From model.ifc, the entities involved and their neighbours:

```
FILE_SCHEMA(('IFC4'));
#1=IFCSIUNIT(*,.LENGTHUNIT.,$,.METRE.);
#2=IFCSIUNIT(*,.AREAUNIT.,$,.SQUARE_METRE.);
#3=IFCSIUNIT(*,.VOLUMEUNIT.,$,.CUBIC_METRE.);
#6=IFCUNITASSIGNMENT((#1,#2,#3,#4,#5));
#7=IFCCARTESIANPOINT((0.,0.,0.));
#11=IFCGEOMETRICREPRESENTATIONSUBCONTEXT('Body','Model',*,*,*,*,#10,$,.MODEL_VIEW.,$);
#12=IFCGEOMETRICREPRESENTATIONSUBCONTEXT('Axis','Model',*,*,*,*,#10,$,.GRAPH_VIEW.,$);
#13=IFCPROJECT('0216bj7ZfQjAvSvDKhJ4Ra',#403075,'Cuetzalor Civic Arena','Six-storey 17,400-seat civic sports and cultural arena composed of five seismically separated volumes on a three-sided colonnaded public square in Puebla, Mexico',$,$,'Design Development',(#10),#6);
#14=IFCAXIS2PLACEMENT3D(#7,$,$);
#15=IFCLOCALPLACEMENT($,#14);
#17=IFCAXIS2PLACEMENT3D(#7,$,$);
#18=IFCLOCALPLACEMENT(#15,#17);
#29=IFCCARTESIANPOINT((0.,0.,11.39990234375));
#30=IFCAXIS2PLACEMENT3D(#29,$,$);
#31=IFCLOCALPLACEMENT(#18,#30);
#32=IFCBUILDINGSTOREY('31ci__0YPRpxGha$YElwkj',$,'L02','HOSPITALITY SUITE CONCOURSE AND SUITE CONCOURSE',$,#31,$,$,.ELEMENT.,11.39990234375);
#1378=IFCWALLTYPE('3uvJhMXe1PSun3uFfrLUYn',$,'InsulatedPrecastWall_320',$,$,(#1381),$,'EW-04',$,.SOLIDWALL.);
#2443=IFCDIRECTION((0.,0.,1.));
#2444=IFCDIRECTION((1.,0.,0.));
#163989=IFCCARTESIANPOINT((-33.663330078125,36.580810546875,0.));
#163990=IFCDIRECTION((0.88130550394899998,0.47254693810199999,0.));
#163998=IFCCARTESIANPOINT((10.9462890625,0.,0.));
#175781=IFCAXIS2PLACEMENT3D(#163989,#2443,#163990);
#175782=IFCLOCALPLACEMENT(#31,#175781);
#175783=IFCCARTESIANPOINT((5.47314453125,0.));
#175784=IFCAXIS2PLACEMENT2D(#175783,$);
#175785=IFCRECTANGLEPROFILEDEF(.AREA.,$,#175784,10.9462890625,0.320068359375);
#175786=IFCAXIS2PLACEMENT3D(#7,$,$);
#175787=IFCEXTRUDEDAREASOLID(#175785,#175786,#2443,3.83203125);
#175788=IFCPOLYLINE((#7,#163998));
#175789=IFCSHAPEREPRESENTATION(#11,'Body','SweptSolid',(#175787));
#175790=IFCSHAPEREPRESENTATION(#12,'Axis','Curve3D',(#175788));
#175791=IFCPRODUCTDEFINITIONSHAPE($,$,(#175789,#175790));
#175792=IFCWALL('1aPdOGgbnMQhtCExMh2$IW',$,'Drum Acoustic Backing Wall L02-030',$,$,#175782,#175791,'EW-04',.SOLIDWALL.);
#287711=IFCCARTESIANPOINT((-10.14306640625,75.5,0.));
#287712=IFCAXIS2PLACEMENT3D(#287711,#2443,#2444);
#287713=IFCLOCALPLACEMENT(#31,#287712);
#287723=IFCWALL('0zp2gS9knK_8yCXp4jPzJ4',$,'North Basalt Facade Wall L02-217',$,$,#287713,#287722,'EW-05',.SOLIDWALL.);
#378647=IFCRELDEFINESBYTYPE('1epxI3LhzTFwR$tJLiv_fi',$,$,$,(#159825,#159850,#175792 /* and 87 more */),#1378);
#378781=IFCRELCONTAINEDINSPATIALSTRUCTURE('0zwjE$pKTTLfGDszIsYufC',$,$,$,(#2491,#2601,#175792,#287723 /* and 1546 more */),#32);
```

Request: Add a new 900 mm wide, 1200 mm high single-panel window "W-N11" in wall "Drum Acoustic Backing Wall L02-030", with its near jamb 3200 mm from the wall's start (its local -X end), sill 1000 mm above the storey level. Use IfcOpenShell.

```python
import numpy as np
import ifcopenshell
import ifcopenshell.api.feature
import ifcopenshell.api.geometry
import ifcopenshell.api.root
import ifcopenshell.api.spatial
import ifcopenshell.geom
import ifcopenshell.util.element
import ifcopenshell.util.placement
import ifcopenshell.util.representation
import ifcopenshell.util.shape
import ifcopenshell.util.unit

model = ifcopenshell.open("model.ifc")
unit_scale = ifcopenshell.util.unit.calculate_unit_scale(model)
settings = ifcopenshell.geom.settings()


def volume(element):
    """Net volume in cubic metres, openings subtracted."""
    shape = ifcopenshell.geom.create_shape(settings, element)
    return ifcopenshell.util.shape.get_volume(shape.geometry)


wall = model.by_guid("1aPdOGgbnMQhtCExMh2$IW")
storey = ifcopenshell.util.element.get_container(wall, ifc_class="IfcBuildingStorey")
context = ifcopenshell.util.representation.get_context(model, "Model", "Body", "MODEL_VIEW")
before = volume(wall)

width, height, from_end, sill = 0.9, 1.2, 3.2, 1  # metres

# The wall runs along its own X axis, and the end named is its -X end.
wall_shape = ifcopenshell.geom.create_shape(settings, wall)
x, y, z = ifcopenshell.util.shape.get_vertices(wall_shape.geometry).T
start = x.min() + from_end
face, thickness = float(y.min()), float(y.max() - y.min())
wall_matrix = ifcopenshell.util.placement.get_local_placement(wall.ObjectPlacement)
level = ifcopenshell.util.placement.get_local_placement(storey.ObjectPlacement)[2, 3]


def in_wall(x, y):
    """Placement at x, y metres in the wall's axes, at sill height."""
    matrix = wall_matrix.copy()
    matrix[:, 3] = wall_matrix @ np.array([x / unit_scale, y / unit_scale, 0.0, 1.0])
    matrix[2, 3] = level + sill / unit_scale
    return matrix


# Opening: a box that overshoots both wall faces by 50 mm.
opening = ifcopenshell.api.root.create_entity(model, ifc_class="IfcOpeningElement", predefined_type="OPENING")
box = ifcopenshell.api.geometry.add_wall_representation(
    model, context=context, length=width, height=height, thickness=thickness + 0.1
)
ifcopenshell.api.geometry.assign_representation(model, product=opening, representation=box)
ifcopenshell.api.geometry.edit_object_placement(model, product=opening, matrix=in_wall(start, face - 0.05), is_si=False)
ifcopenshell.api.feature.add_feature(model, feature=opening, element=wall)

window = ifcopenshell.api.root.create_entity(model, ifc_class="IfcWindow", name="W-N11", predefined_type="WINDOW")
window.OverallWidth, window.OverallHeight = width / unit_scale, height / unit_scale
window.PartitioningType = "SINGLE_PANEL"
body = ifcopenshell.api.geometry.add_window_representation(
    model,
    context=context,
    overall_width=window.OverallWidth,
    overall_height=window.OverallHeight,
    partition_type="SINGLE_PANEL",
)
ifcopenshell.api.geometry.assign_representation(model, product=window, representation=body)
ifcopenshell.api.spatial.assign_container(model, products=[window], relating_structure=storey)
ifcopenshell.api.feature.add_filling(model, opening=opening, element=window)

# Centre the window in the wall's thickness.
ifcopenshell.api.geometry.edit_object_placement(model, product=window, matrix=in_wall(start, face), is_si=False)
window_shape = ifcopenshell.geom.create_shape(settings, window)
depth = ifcopenshell.util.shape.get_vertices(window_shape.geometry)[:, 1]
offset = face + thickness / 2 - (depth.min() + depth.max()) / 2
ifcopenshell.api.geometry.edit_object_placement(model, product=window, matrix=in_wall(start, offset), is_si=False)

after = volume(wall)

print(f"wall volume {before:.3f} -> {after:.3f} m3")

model.write("model-out.ifc")
```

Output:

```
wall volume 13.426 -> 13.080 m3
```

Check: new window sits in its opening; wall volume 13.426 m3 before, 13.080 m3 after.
